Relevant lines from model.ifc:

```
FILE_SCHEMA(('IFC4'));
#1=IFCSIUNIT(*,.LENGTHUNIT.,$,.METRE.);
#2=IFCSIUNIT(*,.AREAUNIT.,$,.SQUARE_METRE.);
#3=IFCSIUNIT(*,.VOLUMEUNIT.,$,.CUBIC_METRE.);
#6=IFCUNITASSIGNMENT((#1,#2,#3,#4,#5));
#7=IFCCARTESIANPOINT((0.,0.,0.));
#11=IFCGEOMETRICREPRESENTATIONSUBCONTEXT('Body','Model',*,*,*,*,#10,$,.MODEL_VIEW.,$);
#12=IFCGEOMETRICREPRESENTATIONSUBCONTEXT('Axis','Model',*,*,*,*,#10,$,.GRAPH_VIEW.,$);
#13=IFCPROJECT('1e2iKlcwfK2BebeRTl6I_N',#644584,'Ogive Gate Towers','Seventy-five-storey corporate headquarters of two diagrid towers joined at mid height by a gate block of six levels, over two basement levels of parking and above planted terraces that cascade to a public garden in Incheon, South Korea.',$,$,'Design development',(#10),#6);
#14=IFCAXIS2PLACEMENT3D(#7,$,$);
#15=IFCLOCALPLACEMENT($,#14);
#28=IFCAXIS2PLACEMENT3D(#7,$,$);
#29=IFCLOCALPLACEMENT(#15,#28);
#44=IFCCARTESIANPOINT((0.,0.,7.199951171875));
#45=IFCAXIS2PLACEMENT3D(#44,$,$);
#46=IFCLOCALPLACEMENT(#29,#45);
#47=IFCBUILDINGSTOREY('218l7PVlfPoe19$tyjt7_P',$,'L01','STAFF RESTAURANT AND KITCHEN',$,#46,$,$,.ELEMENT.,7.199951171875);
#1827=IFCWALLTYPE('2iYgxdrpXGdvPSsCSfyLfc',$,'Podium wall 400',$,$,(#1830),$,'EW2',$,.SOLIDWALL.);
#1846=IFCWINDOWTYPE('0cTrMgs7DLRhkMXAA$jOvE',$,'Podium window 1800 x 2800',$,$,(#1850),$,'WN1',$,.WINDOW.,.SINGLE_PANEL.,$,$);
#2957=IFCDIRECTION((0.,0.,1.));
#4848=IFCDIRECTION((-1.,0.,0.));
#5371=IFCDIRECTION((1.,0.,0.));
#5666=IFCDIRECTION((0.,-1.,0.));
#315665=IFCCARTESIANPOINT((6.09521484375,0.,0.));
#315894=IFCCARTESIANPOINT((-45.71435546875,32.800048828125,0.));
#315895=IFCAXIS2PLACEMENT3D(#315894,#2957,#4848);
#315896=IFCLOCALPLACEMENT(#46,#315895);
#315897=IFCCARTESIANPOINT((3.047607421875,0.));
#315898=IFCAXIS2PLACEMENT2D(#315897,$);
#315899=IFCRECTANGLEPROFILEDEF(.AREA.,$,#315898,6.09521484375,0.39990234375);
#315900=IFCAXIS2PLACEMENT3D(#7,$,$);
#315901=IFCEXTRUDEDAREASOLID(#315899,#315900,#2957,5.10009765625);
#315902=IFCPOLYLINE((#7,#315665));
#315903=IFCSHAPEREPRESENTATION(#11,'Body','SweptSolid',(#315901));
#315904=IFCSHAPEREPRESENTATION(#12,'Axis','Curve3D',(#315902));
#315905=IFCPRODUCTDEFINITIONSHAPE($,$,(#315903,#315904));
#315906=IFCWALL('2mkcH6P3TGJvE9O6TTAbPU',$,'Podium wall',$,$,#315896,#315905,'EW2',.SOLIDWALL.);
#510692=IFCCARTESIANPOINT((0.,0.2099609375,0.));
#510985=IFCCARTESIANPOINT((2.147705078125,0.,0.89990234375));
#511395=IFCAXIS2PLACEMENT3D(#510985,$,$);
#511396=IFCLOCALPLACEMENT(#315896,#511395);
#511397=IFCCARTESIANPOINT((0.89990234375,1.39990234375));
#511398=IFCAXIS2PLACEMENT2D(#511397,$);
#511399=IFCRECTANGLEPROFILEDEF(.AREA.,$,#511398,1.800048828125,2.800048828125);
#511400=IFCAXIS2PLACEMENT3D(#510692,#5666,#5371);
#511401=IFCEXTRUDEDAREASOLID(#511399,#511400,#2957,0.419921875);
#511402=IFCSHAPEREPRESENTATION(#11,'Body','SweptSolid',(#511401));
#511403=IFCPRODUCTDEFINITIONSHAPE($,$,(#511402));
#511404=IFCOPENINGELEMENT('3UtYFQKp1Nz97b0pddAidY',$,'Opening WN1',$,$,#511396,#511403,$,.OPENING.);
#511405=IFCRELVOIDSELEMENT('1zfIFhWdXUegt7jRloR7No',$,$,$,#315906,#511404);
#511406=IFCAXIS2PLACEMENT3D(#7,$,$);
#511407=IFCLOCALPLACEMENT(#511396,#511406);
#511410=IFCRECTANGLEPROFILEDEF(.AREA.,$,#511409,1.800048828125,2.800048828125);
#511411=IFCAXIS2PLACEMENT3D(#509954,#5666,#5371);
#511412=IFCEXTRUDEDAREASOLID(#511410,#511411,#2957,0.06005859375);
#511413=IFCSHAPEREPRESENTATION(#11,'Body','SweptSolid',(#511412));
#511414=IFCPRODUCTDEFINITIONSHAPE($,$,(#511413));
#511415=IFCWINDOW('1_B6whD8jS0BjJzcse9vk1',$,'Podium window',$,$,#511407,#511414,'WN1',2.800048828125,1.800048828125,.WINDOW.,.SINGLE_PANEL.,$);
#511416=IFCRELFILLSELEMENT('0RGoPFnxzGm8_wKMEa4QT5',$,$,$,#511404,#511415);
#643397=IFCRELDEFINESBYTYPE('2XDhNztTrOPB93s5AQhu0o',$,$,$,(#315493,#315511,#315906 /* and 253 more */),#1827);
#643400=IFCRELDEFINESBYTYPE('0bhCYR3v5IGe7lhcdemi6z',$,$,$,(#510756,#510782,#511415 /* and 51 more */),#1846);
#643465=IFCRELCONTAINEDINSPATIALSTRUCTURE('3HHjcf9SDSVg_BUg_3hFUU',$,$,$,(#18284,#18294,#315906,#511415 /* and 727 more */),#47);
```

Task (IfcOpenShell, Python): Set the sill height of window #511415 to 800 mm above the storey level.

```python
import numpy as np
import ifcopenshell
import ifcopenshell.api.geometry
import ifcopenshell.geom
import ifcopenshell.util.element
import ifcopenshell.util.placement
import ifcopenshell.util.shape
import ifcopenshell.util.unit

model = ifcopenshell.open("model.ifc")
unit_scale = ifcopenshell.util.unit.calculate_unit_scale(model)

window = model.by_guid("1_B6whD8jS0BjJzcse9vk1")
opening = window.FillsVoids[0].RelatingOpeningElement
storey = ifcopenshell.util.element.get_container(window, ifc_class="IfcBuildingStorey")
level = ifcopenshell.util.placement.get_local_placement(storey.ObjectPlacement)[2, 3]

# The opening's origin need not be at the sill, so measure its lowest point.
shape = ifcopenshell.geom.create_shape(ifcopenshell.geom.settings(), opening)
bottom = ifcopenshell.util.shape.get_shape_bottom_elevation(shape, shape.geometry) / unit_scale
dz = level + 0.8 / unit_scale - bottom

shift = np.array([0.0, 0.0, dz])
# The window is placed relative to its opening, so it follows when the opening moves.
matrix = ifcopenshell.util.placement.get_local_placement(opening.ObjectPlacement)
matrix[:3, 3] += shift
ifcopenshell.api.geometry.edit_object_placement(
    model, product=opening, matrix=matrix, is_si=False, should_transform_children=True
)

print(f"moved by {dz * unit_scale:+.3f} m")

model.write("model_rev.ifc")
```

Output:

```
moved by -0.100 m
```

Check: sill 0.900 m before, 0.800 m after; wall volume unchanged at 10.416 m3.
